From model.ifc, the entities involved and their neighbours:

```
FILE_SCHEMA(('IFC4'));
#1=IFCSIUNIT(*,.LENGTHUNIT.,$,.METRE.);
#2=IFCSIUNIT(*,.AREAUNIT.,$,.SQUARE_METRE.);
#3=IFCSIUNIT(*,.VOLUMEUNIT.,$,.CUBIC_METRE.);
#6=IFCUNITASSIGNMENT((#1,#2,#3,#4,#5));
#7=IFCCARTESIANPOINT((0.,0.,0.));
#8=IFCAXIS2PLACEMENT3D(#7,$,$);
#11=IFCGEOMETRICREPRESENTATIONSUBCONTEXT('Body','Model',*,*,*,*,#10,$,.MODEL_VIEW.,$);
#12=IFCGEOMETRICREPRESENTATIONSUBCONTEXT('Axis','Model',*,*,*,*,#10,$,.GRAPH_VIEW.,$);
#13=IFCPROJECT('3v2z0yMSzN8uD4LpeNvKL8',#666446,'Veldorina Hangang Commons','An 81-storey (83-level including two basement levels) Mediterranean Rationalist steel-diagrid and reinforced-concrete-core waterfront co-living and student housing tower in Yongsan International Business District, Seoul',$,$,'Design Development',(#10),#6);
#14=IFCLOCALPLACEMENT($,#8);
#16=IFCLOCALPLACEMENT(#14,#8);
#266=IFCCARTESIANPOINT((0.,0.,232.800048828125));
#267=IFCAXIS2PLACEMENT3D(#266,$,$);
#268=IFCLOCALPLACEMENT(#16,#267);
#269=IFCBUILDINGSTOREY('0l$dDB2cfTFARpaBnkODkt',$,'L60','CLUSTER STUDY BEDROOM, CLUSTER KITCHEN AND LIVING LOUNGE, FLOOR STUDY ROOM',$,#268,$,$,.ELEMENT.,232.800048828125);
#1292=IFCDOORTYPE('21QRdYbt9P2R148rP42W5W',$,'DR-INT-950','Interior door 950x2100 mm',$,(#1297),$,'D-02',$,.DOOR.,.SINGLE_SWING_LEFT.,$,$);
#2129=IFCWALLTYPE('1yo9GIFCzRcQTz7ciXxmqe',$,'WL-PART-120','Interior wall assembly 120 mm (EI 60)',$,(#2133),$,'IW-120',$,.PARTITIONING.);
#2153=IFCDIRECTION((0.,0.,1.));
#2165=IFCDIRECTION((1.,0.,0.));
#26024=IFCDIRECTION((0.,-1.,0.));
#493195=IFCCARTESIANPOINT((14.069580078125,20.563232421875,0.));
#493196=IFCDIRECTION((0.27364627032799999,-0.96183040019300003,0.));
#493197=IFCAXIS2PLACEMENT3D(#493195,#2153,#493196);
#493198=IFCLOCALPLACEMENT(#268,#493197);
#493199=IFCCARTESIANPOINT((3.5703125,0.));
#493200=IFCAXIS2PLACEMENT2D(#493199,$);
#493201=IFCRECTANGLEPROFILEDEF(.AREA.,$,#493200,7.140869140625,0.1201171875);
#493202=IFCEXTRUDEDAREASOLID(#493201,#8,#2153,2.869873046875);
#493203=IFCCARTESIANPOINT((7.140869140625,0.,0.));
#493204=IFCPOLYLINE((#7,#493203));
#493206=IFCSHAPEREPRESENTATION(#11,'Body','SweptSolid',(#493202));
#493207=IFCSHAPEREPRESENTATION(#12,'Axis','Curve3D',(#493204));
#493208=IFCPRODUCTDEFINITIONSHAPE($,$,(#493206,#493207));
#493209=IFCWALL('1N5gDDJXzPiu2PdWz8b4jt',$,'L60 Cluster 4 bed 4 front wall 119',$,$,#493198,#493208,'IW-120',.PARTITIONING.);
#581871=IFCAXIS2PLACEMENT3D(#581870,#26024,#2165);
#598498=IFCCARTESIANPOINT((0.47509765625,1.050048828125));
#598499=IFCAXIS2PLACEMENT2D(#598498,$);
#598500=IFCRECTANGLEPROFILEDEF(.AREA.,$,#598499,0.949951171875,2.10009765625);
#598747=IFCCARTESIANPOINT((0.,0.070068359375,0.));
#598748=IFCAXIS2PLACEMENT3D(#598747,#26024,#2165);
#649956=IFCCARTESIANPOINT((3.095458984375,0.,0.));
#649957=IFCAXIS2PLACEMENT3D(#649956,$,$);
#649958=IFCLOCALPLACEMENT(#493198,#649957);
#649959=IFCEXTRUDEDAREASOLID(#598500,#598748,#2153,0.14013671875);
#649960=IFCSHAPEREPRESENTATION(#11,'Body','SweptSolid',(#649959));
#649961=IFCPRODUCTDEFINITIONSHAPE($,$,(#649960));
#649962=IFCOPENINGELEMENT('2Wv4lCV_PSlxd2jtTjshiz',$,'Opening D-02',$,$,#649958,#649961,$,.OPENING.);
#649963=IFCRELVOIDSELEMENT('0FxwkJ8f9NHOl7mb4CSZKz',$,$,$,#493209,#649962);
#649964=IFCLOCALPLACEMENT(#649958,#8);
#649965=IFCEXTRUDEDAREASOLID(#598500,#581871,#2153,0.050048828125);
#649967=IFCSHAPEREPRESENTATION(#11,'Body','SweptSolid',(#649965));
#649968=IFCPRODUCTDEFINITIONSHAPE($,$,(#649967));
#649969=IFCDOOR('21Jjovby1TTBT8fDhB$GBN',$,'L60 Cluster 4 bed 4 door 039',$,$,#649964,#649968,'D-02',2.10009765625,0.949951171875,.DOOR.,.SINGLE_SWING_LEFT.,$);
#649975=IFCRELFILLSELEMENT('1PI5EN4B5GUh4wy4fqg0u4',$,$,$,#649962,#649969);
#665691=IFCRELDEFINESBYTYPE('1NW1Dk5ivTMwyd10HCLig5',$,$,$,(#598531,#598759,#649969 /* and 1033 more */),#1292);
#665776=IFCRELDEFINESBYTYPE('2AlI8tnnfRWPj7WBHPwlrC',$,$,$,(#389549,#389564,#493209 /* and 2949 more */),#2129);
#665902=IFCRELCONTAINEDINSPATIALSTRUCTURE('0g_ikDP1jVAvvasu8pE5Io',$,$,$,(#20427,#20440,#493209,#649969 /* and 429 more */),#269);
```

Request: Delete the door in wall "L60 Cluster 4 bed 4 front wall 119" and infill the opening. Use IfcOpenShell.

```python
import ifcopenshell
import ifcopenshell.api.feature
import ifcopenshell.api.root
import ifcopenshell.geom
import ifcopenshell.util.shape

model = ifcopenshell.open("model.ifc")
settings = ifcopenshell.geom.settings()


def volume(element):
    """Net volume in cubic metres, openings subtracted."""
    shape = ifcopenshell.geom.create_shape(settings, element)
    return ifcopenshell.util.shape.get_volume(shape.geometry)


door = model.by_guid("21Jjovby1TTBT8fDhB$GBN")
opening = door.FillsVoids[0].RelatingOpeningElement
wall = opening.VoidsElements[0].RelatingBuildingElement
before = volume(wall)

ifcopenshell.api.root.remove_product(model, product=door)
ifcopenshell.api.feature.remove_feature(model, feature=opening)

after = volume(wall)

print(f"wall volume {before:.3f} -> {after:.3f} m3")

model.write("model-out.ifc")
```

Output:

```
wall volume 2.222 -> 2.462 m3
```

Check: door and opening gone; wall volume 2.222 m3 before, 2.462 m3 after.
